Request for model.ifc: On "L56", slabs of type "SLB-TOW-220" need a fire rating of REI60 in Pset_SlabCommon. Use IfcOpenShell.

First a look at what the model holds.

```python
import ifcopenshell
import ifcopenshell.util.element

model = ifcopenshell.open("model.ifc")
print(model.schema)
storey = next(s for s in model.by_type("IfcBuildingStorey") if s.Name == "L56")
slabs = [e for e in ifcopenshell.util.element.get_decomposition(storey) if e.is_a("IfcSlab")]
seen = {}
for e in slabs:
    element_type = ifcopenshell.util.element.get_type(e)
    key = (element_type.Name if element_type != e and element_type else None, ifcopenshell.util.element.get_pset(e, "Pset_SlabCommon", "FireRating"))
    seen[key] = seen.get(key, 0) + 1
for (name, value), count in sorted(seen.items(), key=str):
    print(count, "x", name, "|", value)
```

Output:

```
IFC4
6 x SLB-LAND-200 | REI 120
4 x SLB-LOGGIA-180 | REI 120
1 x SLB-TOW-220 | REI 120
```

```python
import ifcopenshell
import ifcopenshell.api.pset
import ifcopenshell.util.element

model = ifcopenshell.open("model.ifc")

storey = next(s for s in model.by_type("IfcBuildingStorey") if s.Name == "L56")
slabs = [e for e in ifcopenshell.util.element.get_decomposition(storey) if e.is_a("IfcSlab")]

count = 0
for e in slabs:
    element_type = ifcopenshell.util.element.get_type(e)
    if element_type in (None, e) or element_type.Name != "SLB-TOW-220":
        continue
    found = ifcopenshell.util.element.get_pset(e, "Pset_SlabCommon", should_inherit=False)
    if found:
        pset = model.by_id(found["id"])
        if len(ifcopenshell.util.element.get_elements_by_pset(pset)) > 1:
            pset = ifcopenshell.api.pset.unshare_pset(model, products=[e], pset=pset)[0]
    else:
        pset = ifcopenshell.api.pset.add_pset(model, product=e, name="Pset_SlabCommon")
    ifcopenshell.api.pset.edit_pset(model, pset=pset, properties={"FireRating": "REI60"})
    count += 1

print(count, "slabs updated")

model.write("model-out.ifc")
```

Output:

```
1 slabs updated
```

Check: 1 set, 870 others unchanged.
